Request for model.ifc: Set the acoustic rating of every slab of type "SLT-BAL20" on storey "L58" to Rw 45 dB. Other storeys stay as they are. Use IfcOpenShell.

First a look at what the model holds.

```python
import ifcopenshell
import ifcopenshell.util.element

model = ifcopenshell.open("model.ifc")
print(model.schema)
storey = next(s for s in model.by_type("IfcBuildingStorey") if s.Name == "L58")
slabs = [e for e in ifcopenshell.util.element.get_decomposition(storey) if e.is_a("IfcSlab")]
seen = {}
for e in slabs:
    element_type = ifcopenshell.util.element.get_type(e)
    key = (element_type.Name if element_type != e and element_type else None, ifcopenshell.util.element.get_pset(e, "Pset_SlabCommon", "AcousticRating"))
    seen[key] = seen.get(key, 0) + 1
for (name, value), count in sorted(seen.items(), key=str):
    print(count, "x", name, "|", value)
```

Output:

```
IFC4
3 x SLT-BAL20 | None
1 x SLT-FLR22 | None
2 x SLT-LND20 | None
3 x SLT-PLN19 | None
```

```python
import ifcopenshell
import ifcopenshell.api.pset
import ifcopenshell.util.element

model = ifcopenshell.open("model.ifc")

storey = next(s for s in model.by_type("IfcBuildingStorey") if s.Name == "L58")
slabs = [e for e in ifcopenshell.util.element.get_decomposition(storey) if e.is_a("IfcSlab")]

count = 0
for e in slabs:
    element_type = ifcopenshell.util.element.get_type(e)
    if element_type in (None, e) or element_type.Name != "SLT-BAL20":
        continue
    # add_pset returns the element's existing set when there is one.
    pset = ifcopenshell.api.pset.add_pset(model, product=e, name="Pset_SlabCommon")
    ifcopenshell.api.pset.edit_pset(model, pset=pset, properties={"AcousticRating": "Rw 45 dB"})
    count += 1

print(count, "slabs updated")

model.write("model_updated.ifc")
```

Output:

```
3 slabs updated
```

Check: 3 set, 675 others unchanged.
